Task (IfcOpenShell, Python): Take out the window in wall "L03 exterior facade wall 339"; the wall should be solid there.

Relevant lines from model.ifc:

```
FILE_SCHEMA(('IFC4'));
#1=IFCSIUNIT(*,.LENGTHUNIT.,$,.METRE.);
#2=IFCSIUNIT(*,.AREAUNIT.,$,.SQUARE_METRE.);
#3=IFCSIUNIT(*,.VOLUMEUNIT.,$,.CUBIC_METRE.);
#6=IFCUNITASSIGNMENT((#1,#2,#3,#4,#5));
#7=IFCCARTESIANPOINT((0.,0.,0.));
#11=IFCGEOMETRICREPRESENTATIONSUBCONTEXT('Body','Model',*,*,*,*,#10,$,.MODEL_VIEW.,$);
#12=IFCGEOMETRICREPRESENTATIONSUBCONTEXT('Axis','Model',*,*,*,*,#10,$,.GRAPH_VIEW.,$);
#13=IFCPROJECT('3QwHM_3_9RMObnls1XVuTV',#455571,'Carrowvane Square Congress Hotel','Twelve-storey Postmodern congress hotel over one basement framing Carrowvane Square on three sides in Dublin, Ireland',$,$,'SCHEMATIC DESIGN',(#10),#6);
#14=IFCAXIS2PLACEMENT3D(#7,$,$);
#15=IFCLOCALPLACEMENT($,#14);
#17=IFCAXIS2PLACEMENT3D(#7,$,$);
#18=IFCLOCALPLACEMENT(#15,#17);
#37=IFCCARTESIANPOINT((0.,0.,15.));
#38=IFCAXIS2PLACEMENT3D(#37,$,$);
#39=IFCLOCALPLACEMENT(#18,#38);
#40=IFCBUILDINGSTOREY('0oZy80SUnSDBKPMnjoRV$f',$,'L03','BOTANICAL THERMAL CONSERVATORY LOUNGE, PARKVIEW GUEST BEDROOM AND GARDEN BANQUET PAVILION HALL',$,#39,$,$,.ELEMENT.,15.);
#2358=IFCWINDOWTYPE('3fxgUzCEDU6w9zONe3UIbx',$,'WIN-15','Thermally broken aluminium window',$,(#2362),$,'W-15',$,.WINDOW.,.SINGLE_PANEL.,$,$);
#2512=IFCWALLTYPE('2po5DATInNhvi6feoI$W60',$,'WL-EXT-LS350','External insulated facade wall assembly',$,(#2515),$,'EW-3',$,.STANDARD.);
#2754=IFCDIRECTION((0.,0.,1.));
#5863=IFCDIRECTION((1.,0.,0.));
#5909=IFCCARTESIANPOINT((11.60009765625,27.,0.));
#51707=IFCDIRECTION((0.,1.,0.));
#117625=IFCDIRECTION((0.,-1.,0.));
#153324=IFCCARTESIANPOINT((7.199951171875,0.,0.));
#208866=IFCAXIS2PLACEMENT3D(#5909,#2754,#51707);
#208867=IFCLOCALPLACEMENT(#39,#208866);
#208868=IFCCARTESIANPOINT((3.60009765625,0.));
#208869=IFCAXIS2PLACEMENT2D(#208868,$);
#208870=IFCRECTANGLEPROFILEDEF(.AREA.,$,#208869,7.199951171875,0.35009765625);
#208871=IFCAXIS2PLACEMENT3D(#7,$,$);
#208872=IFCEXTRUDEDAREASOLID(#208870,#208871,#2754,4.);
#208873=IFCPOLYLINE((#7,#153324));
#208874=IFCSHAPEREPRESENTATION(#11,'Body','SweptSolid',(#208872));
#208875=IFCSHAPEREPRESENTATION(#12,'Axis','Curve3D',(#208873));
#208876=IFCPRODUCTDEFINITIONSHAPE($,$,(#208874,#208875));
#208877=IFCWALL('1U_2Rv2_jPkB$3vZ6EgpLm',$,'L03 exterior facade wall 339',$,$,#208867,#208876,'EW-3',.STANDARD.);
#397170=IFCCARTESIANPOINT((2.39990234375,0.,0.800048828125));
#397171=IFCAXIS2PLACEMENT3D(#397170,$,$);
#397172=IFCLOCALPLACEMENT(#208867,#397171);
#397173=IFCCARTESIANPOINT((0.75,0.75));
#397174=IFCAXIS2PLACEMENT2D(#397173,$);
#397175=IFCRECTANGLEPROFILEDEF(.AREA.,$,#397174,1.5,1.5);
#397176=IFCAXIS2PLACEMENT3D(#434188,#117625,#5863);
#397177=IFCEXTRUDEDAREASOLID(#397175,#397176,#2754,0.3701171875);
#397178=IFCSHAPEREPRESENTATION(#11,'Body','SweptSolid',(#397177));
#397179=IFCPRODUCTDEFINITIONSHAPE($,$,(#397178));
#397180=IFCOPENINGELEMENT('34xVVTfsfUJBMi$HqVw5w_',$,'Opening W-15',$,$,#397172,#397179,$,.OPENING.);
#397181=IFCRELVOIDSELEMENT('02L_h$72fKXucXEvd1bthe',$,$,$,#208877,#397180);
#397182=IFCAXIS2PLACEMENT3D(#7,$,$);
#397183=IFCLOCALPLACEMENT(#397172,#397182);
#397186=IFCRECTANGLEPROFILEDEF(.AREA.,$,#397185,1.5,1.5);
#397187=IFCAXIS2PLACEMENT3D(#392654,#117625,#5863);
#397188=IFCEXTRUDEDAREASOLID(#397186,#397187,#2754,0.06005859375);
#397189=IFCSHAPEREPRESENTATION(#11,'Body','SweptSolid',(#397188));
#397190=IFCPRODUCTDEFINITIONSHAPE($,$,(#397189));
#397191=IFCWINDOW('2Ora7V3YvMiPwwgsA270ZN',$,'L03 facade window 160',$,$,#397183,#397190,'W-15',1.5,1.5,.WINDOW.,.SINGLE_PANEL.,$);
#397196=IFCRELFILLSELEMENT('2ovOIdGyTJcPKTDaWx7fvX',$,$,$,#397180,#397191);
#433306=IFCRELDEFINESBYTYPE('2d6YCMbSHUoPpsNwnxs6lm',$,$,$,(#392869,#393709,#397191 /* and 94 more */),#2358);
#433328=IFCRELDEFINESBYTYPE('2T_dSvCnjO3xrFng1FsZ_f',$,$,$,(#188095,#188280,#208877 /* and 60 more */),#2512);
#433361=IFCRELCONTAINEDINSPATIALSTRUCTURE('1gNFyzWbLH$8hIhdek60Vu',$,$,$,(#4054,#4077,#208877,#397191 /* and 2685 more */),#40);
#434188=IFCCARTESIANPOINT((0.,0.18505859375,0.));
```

```python
import ifcopenshell
import ifcopenshell.api.feature
import ifcopenshell.api.root
import ifcopenshell.geom
import ifcopenshell.util.shape

model = ifcopenshell.open("model.ifc")
settings = ifcopenshell.geom.settings()


def volume(element):
    """Net volume in cubic metres, openings subtracted."""
    shape = ifcopenshell.geom.create_shape(settings, element)
    return ifcopenshell.util.shape.get_volume(shape.geometry)


window = model.by_guid("2Ora7V3YvMiPwwgsA270ZN")
opening = window.FillsVoids[0].RelatingOpeningElement
wall = opening.VoidsElements[0].RelatingBuildingElement
before = volume(wall)

ifcopenshell.api.root.remove_product(model, product=window)
ifcopenshell.api.feature.remove_feature(model, feature=opening)

after = volume(wall)

print(f"wall volume {before:.3f} -> {after:.3f} m3")

model.write("model_updated.ifc")
```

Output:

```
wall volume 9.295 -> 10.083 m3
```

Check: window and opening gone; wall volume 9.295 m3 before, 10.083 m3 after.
